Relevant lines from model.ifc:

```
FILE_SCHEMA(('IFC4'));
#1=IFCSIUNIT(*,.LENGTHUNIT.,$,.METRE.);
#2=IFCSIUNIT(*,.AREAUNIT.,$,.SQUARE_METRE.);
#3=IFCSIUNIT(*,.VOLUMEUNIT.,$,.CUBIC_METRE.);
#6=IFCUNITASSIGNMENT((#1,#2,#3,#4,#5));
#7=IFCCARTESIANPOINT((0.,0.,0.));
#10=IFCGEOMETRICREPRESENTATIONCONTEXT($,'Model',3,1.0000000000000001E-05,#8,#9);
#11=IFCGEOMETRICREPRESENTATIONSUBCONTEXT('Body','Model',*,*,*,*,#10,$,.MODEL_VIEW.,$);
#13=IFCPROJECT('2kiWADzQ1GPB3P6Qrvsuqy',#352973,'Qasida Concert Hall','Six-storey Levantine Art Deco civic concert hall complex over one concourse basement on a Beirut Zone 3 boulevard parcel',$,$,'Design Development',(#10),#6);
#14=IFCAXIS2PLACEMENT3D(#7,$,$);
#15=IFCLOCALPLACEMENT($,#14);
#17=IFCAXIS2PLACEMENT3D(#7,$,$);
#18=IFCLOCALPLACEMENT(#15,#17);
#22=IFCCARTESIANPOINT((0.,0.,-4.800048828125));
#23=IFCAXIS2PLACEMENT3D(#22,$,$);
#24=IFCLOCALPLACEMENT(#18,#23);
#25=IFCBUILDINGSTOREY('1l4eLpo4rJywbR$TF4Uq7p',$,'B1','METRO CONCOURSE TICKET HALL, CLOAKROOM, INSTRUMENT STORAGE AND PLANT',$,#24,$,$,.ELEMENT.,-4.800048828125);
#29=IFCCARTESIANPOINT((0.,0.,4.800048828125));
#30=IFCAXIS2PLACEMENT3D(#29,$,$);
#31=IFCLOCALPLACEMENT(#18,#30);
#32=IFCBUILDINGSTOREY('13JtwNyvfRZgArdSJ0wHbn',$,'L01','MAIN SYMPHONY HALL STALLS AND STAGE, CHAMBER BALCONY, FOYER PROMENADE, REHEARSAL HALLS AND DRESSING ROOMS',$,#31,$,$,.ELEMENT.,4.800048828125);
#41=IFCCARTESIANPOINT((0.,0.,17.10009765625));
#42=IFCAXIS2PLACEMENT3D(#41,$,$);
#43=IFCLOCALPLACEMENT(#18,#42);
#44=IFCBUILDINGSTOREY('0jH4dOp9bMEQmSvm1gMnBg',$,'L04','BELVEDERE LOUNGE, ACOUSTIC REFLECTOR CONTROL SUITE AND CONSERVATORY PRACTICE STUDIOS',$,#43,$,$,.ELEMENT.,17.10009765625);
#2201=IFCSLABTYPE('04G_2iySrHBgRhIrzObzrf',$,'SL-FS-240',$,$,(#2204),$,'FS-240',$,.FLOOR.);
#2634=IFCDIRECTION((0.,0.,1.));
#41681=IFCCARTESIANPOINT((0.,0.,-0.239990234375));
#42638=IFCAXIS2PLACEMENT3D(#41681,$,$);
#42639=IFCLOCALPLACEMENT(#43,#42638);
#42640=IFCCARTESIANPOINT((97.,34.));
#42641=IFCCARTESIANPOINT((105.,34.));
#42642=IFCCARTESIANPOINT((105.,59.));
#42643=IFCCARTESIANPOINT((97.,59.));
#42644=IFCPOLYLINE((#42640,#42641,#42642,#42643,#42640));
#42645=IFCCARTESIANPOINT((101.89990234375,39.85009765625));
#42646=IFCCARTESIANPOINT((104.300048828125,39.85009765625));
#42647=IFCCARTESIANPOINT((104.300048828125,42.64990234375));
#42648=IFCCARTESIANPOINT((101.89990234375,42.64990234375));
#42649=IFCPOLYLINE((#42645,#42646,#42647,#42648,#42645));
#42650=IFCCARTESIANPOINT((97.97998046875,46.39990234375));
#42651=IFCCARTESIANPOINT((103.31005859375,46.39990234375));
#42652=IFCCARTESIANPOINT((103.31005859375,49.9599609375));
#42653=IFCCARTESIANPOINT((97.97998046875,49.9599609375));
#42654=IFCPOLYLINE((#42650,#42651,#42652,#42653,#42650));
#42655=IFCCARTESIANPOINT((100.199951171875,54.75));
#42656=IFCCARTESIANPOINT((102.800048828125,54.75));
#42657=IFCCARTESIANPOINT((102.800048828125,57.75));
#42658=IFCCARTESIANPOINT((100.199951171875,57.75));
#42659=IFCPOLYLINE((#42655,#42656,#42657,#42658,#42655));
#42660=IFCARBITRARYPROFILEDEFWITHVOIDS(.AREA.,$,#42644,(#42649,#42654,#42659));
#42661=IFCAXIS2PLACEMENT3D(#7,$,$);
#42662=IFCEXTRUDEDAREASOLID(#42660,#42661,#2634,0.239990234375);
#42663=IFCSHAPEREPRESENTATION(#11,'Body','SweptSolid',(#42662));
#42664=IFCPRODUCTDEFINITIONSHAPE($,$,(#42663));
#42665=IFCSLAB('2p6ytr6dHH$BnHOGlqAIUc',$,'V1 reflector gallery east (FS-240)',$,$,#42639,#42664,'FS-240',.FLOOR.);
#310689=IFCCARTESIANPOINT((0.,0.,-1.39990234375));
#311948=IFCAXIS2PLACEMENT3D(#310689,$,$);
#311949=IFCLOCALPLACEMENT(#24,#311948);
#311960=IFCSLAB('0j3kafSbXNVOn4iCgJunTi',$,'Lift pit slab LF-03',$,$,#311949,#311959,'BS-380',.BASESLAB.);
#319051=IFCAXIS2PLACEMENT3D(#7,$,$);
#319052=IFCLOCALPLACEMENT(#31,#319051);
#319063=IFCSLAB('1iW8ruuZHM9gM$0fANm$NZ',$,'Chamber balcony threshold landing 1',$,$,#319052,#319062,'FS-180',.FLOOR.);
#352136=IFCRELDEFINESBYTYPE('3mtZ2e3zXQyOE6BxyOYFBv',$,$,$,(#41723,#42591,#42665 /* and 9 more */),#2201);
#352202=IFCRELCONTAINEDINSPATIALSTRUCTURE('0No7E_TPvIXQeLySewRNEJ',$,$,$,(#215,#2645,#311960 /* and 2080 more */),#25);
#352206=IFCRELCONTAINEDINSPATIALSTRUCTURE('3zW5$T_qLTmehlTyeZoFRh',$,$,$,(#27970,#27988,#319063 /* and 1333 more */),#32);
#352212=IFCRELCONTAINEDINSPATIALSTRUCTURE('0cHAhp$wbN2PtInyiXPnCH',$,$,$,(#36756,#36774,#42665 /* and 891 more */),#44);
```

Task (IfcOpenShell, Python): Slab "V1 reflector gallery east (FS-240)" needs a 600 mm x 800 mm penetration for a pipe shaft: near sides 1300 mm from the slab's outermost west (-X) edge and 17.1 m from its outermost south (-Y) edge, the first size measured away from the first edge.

```python
import numpy as np
import ifcopenshell
import ifcopenshell.api.feature
import ifcopenshell.api.geometry
import ifcopenshell.api.root
import ifcopenshell.geom
import ifcopenshell.util.placement
import ifcopenshell.util.representation
import ifcopenshell.util.shape
import ifcopenshell.util.unit

model = ifcopenshell.open("model.ifc")
unit_scale = ifcopenshell.util.unit.calculate_unit_scale(model)
settings = ifcopenshell.geom.settings()


def volume(element):
    """Net volume in cubic metres, openings subtracted."""
    shape = ifcopenshell.geom.create_shape(settings, element)
    return ifcopenshell.util.shape.get_volume(shape.geometry)


slab = model.by_guid("2p6ytr6dHH$BnHOGlqAIUc")
before = volume(slab)

# Extent in the slab's own axes, in metres. The edges named are its -X and -Y sides.
slab_shape = ifcopenshell.geom.create_shape(settings, slab)
vertices = ifcopenshell.util.shape.get_vertices(slab_shape.geometry)
x_min, y_min, bottom = vertices.min(axis=0)
top = vertices[:, 2].max()

opening = ifcopenshell.api.root.create_entity(model, ifc_class="IfcOpeningElement", name="Pipe shaft opening", predefined_type="OPENING")
context = ifcopenshell.util.representation.get_context(model, "Model", "Body", "MODEL_VIEW")
width, depth = 0.6, 0.8
outline = [(0.0, 0.0), (width, 0.0), (width, depth), (0.0, depth), (0.0, 0.0)]
# Overshoot both faces by 50 mm so the cut is clean.
shape = ifcopenshell.api.geometry.add_slab_representation(
    model, context=context, depth=top - bottom + 0.1, polyline=outline
)
ifcopenshell.api.geometry.assign_representation(model, product=opening, representation=shape)

matrix = ifcopenshell.util.placement.get_local_placement(slab.ObjectPlacement)
matrix[:, 3] = matrix @ np.append(np.array([x_min + 1.3, y_min + 17.1, bottom - 0.05]) / unit_scale, 1.0)
ifcopenshell.api.geometry.edit_object_placement(model, product=opening, matrix=matrix, is_si=False)
ifcopenshell.api.feature.add_feature(model, feature=opening, element=slab)

after = volume(slab)

print(f"slab volume {before:.3f} -> {after:.3f} m3")

model.write("model_updated.ifc")
```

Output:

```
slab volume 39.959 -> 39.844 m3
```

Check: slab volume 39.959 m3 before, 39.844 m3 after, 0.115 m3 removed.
